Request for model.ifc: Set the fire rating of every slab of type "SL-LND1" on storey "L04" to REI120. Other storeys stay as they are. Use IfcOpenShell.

First a look at what the model holds.

```python
import ifcopenshell
import ifcopenshell.util.element

model = ifcopenshell.open("model.ifc")
print(model.schema)
storey = next(s for s in model.by_type("IfcBuildingStorey") if s.Name == "L04")
slabs = [e for e in ifcopenshell.util.element.get_decomposition(storey) if e.is_a("IfcSlab")]
seen = {}
for e in slabs:
    element_type = ifcopenshell.util.element.get_type(e)
    key = (element_type.Name if element_type != e and element_type else None, ifcopenshell.util.element.get_pset(e, "Pset_SlabCommon", "FireRating"))
    seen[key] = seen.get(key, 0) + 1
for (name, value), count in sorted(seen.items(), key=str):
    print(count, "x", name, "|", value)
```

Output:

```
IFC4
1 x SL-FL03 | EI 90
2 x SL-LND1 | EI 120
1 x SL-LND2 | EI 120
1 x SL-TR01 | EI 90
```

```python
import ifcopenshell
import ifcopenshell.api.pset
import ifcopenshell.util.element

model = ifcopenshell.open("model.ifc")

storey = next(s for s in model.by_type("IfcBuildingStorey") if s.Name == "L04")
slabs = [e for e in ifcopenshell.util.element.get_decomposition(storey) if e.is_a("IfcSlab")]

count = 0
for e in slabs:
    element_type = ifcopenshell.util.element.get_type(e)
    if element_type in (None, e) or element_type.Name != "SL-LND1":
        continue
    # add_pset returns the element's existing set when there is one.
    pset = ifcopenshell.api.pset.add_pset(model, product=e, name="Pset_SlabCommon")
    ifcopenshell.api.pset.edit_pset(model, pset=pset, properties={"FireRating": "REI120"})
    count += 1

print(count, "slabs updated")

model.write("model_rev.ifc")
```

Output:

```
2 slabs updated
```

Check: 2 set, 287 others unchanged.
